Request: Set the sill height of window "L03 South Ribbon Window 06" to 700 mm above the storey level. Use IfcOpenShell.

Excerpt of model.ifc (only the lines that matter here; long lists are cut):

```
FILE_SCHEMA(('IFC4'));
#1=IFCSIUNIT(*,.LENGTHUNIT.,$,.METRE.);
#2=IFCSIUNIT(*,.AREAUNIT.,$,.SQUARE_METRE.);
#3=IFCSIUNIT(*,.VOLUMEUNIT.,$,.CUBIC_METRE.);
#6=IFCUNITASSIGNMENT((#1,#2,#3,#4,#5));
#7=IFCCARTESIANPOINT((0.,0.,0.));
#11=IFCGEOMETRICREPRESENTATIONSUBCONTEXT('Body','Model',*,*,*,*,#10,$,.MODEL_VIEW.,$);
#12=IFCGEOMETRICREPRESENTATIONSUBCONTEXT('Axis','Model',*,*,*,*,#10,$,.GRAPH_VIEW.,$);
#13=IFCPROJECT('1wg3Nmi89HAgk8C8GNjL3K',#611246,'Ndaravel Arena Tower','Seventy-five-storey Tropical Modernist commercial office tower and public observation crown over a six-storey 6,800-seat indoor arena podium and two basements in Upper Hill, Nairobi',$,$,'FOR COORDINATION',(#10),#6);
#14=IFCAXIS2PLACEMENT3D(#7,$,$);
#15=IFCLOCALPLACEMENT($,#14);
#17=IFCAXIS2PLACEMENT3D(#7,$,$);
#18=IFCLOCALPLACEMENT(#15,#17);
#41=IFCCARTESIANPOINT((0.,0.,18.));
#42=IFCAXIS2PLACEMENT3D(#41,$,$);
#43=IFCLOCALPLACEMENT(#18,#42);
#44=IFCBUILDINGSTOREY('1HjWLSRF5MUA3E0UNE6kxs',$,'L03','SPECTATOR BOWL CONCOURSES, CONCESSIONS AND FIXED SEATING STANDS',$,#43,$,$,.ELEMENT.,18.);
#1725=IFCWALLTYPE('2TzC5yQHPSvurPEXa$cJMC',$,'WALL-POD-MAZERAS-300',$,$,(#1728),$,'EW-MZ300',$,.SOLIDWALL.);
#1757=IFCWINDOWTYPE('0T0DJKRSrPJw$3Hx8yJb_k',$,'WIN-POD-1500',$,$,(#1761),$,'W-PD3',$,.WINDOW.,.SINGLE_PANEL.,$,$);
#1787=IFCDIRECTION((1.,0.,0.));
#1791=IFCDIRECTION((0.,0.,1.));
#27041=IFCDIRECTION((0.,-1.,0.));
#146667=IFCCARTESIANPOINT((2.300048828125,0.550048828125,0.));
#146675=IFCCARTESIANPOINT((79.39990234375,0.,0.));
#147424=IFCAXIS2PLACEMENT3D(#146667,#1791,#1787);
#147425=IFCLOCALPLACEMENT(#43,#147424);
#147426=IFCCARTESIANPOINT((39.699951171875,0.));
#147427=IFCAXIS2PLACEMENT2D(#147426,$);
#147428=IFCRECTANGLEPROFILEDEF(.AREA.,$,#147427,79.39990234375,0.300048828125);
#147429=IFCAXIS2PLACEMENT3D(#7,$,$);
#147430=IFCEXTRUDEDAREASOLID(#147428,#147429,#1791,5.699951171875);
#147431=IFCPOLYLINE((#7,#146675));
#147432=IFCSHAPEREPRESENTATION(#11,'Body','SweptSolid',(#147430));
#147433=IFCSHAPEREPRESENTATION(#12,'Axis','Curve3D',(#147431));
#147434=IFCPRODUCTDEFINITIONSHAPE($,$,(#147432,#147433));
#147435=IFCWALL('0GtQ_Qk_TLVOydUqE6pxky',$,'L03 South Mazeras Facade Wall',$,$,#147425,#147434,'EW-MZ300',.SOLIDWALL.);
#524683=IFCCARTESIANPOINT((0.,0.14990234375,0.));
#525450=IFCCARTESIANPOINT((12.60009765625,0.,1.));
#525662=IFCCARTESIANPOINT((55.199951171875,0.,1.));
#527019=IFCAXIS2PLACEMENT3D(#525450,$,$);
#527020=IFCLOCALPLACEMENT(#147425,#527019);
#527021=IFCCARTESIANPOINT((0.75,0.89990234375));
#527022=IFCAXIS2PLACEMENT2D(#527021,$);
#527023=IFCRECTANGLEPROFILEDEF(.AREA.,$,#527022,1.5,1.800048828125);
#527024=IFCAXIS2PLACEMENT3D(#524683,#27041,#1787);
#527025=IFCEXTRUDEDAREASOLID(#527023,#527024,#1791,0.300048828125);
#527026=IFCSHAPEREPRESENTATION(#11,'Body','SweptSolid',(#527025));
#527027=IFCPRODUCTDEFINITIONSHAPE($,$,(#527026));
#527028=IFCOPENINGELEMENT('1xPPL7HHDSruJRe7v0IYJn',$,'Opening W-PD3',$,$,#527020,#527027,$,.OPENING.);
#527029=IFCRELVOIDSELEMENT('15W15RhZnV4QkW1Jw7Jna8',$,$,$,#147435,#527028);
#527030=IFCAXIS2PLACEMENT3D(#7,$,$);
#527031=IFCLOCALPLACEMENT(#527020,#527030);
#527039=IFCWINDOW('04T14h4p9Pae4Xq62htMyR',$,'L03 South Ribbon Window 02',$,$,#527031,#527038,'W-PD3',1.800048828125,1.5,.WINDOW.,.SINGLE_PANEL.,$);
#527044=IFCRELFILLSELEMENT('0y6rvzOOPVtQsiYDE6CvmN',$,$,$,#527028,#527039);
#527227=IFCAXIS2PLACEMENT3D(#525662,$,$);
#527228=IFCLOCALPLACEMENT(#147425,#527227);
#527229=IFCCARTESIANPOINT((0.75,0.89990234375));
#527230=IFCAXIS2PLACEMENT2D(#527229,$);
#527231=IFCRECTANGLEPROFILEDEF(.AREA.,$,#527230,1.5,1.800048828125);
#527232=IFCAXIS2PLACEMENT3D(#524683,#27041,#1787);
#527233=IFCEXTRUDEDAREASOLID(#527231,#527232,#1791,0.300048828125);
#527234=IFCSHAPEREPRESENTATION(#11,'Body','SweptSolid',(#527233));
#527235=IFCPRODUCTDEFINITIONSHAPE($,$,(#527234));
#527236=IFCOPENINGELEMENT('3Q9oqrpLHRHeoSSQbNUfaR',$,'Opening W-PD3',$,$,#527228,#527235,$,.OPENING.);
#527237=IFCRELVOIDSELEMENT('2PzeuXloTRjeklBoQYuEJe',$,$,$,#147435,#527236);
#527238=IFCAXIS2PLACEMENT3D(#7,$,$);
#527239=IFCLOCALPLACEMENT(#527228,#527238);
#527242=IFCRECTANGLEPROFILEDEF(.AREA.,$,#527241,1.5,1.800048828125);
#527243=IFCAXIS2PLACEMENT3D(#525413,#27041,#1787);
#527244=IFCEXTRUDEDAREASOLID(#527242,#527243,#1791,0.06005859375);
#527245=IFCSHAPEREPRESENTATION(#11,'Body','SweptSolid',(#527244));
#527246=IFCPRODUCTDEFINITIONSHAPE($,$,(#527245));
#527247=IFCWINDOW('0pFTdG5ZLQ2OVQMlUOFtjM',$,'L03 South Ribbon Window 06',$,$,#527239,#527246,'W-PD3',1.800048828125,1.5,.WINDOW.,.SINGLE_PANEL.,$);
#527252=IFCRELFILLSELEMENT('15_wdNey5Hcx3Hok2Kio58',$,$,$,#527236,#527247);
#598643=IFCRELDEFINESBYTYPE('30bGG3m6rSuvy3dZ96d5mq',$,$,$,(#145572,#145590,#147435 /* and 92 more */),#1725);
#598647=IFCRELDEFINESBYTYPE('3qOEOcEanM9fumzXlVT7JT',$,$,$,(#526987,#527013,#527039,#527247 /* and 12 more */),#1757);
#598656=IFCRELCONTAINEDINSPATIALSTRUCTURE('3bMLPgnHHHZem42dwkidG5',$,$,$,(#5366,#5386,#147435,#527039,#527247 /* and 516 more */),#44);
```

```python
import numpy as np
import ifcopenshell
import ifcopenshell.api.geometry
import ifcopenshell.geom
import ifcopenshell.util.element
import ifcopenshell.util.placement
import ifcopenshell.util.shape
import ifcopenshell.util.unit

model = ifcopenshell.open("model.ifc")
unit_scale = ifcopenshell.util.unit.calculate_unit_scale(model)

window = model.by_id(527247)
opening = window.FillsVoids[0].RelatingOpeningElement
storey = ifcopenshell.util.element.get_container(window, ifc_class="IfcBuildingStorey")
level = ifcopenshell.util.placement.get_local_placement(storey.ObjectPlacement)[2, 3]

# The opening's origin need not be at the sill, so measure its lowest point.
shape = ifcopenshell.geom.create_shape(ifcopenshell.geom.settings(), opening)
bottom = ifcopenshell.util.shape.get_shape_bottom_elevation(shape, shape.geometry) / unit_scale
dz = level + 0.7 / unit_scale - bottom

shift = np.array([0.0, 0.0, dz])
# The window is placed relative to its opening, so it follows when the opening moves.
matrix = ifcopenshell.util.placement.get_local_placement(opening.ObjectPlacement)
matrix[:3, 3] += shift
ifcopenshell.api.geometry.edit_object_placement(
    model, product=opening, matrix=matrix, is_si=False, should_transform_children=True
)

print(f"moved by {dz * unit_scale:+.3f} m")

model.write("model-out.ifc")
```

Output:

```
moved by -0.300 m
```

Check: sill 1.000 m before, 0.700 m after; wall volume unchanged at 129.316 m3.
